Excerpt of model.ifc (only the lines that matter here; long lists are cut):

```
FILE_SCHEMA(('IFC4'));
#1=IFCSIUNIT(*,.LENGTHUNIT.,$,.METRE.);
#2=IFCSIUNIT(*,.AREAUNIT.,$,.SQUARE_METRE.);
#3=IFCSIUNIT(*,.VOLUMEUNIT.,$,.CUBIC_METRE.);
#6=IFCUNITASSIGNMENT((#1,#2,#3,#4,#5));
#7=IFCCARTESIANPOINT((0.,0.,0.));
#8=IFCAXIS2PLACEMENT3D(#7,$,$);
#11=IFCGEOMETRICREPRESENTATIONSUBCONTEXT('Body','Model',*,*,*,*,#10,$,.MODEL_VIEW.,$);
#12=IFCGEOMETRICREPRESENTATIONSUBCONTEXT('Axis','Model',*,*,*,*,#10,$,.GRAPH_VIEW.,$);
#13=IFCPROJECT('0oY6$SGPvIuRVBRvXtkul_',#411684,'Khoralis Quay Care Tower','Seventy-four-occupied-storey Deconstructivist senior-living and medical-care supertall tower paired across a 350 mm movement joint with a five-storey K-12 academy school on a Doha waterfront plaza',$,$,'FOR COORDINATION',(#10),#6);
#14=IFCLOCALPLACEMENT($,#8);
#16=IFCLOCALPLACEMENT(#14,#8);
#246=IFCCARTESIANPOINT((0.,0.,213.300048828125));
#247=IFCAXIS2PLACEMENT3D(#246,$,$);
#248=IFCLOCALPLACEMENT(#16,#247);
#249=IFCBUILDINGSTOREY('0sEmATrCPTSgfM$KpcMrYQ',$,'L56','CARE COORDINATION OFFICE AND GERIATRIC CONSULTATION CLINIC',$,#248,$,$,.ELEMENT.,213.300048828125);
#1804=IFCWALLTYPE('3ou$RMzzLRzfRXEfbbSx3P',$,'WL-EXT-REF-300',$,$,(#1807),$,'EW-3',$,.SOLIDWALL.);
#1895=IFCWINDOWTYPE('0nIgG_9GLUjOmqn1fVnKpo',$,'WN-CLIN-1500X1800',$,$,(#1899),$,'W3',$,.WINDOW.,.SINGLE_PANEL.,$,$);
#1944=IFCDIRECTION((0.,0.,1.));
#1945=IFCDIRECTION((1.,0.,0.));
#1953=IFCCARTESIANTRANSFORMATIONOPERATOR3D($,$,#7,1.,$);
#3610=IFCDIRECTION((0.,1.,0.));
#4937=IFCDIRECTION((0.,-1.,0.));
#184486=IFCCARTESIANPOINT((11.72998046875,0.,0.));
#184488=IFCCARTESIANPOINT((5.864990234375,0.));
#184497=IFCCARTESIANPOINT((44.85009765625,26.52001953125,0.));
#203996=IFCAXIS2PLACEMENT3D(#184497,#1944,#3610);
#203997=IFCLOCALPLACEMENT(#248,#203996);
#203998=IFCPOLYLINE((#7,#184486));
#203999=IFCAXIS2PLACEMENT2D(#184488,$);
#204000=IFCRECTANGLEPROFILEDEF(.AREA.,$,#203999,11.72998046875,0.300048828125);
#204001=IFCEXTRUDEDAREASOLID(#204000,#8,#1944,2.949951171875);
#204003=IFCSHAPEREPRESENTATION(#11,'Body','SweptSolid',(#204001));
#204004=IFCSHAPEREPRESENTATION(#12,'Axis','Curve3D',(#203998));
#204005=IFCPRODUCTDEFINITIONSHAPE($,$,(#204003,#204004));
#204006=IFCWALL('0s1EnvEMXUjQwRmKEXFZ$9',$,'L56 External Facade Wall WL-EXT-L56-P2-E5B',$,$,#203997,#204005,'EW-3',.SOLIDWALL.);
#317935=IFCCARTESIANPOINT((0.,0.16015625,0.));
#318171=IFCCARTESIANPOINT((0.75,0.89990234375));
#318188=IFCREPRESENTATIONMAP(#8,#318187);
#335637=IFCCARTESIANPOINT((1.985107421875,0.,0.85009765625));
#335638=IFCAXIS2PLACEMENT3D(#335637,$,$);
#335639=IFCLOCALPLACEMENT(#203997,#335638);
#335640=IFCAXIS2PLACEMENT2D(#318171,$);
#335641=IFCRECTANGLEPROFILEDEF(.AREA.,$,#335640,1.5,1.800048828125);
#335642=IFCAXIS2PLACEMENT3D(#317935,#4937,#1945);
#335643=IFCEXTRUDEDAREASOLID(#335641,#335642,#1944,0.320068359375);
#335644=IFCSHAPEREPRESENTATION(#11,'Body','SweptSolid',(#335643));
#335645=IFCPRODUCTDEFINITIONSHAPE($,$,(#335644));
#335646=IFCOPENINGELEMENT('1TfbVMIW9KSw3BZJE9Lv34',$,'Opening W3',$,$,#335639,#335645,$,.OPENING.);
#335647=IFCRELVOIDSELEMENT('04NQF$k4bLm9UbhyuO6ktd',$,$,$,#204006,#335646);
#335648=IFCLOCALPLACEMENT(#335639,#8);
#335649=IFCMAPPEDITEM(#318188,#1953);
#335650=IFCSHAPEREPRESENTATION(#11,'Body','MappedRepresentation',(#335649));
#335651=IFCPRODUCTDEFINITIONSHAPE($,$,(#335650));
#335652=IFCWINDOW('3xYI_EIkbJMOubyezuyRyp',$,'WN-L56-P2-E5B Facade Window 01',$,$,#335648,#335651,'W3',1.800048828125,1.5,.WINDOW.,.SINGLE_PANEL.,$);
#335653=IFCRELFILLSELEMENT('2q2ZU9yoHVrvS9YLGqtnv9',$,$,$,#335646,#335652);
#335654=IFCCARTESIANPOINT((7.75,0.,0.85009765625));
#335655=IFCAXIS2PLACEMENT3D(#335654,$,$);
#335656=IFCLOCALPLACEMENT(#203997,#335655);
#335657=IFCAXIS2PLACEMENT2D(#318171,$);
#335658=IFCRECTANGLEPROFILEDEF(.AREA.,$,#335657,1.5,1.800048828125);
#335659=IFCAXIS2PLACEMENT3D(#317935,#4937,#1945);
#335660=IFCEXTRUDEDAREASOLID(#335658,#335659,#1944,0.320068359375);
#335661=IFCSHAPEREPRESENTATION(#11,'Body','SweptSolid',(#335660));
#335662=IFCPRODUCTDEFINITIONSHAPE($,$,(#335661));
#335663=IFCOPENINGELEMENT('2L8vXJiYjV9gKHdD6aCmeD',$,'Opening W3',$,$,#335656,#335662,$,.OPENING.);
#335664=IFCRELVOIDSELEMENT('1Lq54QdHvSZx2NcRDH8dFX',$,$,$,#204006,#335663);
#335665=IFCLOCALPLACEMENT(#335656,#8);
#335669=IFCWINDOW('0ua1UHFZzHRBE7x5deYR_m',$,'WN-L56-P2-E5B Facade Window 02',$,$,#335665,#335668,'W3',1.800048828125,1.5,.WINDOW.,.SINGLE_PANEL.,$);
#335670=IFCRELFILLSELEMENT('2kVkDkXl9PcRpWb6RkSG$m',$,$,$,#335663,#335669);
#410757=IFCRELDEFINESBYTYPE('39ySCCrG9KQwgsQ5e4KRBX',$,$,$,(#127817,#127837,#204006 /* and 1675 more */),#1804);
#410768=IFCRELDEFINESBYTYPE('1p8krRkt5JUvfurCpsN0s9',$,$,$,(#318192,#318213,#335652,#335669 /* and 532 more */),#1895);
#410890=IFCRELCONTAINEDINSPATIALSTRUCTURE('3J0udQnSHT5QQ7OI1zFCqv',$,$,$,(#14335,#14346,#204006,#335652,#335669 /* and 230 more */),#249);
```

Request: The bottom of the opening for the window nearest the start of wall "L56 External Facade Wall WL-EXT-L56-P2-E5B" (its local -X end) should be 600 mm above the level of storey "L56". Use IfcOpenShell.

```python
import numpy as np
import ifcopenshell
import ifcopenshell.api.geometry
import ifcopenshell.geom
import ifcopenshell.util.element
import ifcopenshell.util.placement
import ifcopenshell.util.shape
import ifcopenshell.util.unit

model = ifcopenshell.open("model.ifc")
unit_scale = ifcopenshell.util.unit.calculate_unit_scale(model)

window = model.by_id(335652)
opening = window.FillsVoids[0].RelatingOpeningElement
storey = ifcopenshell.util.element.get_container(window, ifc_class="IfcBuildingStorey")
level = ifcopenshell.util.placement.get_local_placement(storey.ObjectPlacement)[2, 3]

# The opening's origin need not be at the sill, so measure its lowest point.
shape = ifcopenshell.geom.create_shape(ifcopenshell.geom.settings(), opening)
bottom = ifcopenshell.util.shape.get_shape_bottom_elevation(shape, shape.geometry) / unit_scale
dz = level + 0.6 / unit_scale - bottom

shift = np.array([0.0, 0.0, dz])
# The window is placed relative to its opening, so it follows when the opening moves.
matrix = ifcopenshell.util.placement.get_local_placement(opening.ObjectPlacement)
matrix[:3, 3] += shift
ifcopenshell.api.geometry.edit_object_placement(
    model, product=opening, matrix=matrix, is_si=False, should_transform_children=True
)

print(f"moved by {dz * unit_scale:+.3f} m")

model.write("model-out.ifc")
```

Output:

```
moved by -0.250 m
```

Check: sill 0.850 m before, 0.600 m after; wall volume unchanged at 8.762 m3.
